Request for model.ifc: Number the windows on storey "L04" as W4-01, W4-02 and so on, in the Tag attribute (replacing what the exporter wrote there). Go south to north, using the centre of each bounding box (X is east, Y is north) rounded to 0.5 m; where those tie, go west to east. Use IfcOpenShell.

First a look at what the model holds.

```python
import ifcopenshell
import ifcopenshell.util.element
import ifcopenshell.util.placement

model = ifcopenshell.open("model.ifc")
print(model.schema)
storey = next(s for s in model.by_type("IfcBuildingStorey") if s.Name == "L04")
windows = [e for e in ifcopenshell.util.element.get_decomposition(storey) if e.is_a("IfcWindow")]
for e in sorted(windows, key=lambda e: e.id()):
    origin = ifcopenshell.util.placement.get_local_placement(e.ObjectPlacement)[:3, 3]
    print(e.id(), e.Tag, e.Name, origin.round(2) + 0.0, sep=" | ")
```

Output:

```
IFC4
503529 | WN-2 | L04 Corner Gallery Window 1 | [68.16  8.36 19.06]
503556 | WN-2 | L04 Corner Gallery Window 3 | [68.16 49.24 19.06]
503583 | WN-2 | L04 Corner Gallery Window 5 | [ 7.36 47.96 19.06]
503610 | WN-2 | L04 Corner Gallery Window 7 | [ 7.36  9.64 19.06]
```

```python
import ifcopenshell
import ifcopenshell.geom
import ifcopenshell.util.element
import ifcopenshell.util.shape

model = ifcopenshell.open("model.ifc")
settings = ifcopenshell.geom.settings()
settings.set("use-world-coords", True)


def centre(element):
    shape = ifcopenshell.geom.create_shape(settings, element)
    return ifcopenshell.util.shape.get_bbox_centroid(shape.geometry)


storey = next(s for s in model.by_type("IfcBuildingStorey") if s.Name == "L04")
windows = [e for e in ifcopenshell.util.element.get_decomposition(storey) if e.is_a("IfcWindow")]

# Insertion points can sit at a corner or the storey origin, so sort by the geometry (in metres).
centres = {e: centre(e) for e in windows}
windows.sort(key=lambda e: (round(centres[e][1] / 0.5), centres[e][0]))

for i, e in enumerate(windows, start=1):
    number = f"W4-{i:02d}"
    e.Tag = number
    print(e.id(), number)

model.write("model-out.ifc")
```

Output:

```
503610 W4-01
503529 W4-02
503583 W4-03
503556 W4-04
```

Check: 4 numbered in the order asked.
